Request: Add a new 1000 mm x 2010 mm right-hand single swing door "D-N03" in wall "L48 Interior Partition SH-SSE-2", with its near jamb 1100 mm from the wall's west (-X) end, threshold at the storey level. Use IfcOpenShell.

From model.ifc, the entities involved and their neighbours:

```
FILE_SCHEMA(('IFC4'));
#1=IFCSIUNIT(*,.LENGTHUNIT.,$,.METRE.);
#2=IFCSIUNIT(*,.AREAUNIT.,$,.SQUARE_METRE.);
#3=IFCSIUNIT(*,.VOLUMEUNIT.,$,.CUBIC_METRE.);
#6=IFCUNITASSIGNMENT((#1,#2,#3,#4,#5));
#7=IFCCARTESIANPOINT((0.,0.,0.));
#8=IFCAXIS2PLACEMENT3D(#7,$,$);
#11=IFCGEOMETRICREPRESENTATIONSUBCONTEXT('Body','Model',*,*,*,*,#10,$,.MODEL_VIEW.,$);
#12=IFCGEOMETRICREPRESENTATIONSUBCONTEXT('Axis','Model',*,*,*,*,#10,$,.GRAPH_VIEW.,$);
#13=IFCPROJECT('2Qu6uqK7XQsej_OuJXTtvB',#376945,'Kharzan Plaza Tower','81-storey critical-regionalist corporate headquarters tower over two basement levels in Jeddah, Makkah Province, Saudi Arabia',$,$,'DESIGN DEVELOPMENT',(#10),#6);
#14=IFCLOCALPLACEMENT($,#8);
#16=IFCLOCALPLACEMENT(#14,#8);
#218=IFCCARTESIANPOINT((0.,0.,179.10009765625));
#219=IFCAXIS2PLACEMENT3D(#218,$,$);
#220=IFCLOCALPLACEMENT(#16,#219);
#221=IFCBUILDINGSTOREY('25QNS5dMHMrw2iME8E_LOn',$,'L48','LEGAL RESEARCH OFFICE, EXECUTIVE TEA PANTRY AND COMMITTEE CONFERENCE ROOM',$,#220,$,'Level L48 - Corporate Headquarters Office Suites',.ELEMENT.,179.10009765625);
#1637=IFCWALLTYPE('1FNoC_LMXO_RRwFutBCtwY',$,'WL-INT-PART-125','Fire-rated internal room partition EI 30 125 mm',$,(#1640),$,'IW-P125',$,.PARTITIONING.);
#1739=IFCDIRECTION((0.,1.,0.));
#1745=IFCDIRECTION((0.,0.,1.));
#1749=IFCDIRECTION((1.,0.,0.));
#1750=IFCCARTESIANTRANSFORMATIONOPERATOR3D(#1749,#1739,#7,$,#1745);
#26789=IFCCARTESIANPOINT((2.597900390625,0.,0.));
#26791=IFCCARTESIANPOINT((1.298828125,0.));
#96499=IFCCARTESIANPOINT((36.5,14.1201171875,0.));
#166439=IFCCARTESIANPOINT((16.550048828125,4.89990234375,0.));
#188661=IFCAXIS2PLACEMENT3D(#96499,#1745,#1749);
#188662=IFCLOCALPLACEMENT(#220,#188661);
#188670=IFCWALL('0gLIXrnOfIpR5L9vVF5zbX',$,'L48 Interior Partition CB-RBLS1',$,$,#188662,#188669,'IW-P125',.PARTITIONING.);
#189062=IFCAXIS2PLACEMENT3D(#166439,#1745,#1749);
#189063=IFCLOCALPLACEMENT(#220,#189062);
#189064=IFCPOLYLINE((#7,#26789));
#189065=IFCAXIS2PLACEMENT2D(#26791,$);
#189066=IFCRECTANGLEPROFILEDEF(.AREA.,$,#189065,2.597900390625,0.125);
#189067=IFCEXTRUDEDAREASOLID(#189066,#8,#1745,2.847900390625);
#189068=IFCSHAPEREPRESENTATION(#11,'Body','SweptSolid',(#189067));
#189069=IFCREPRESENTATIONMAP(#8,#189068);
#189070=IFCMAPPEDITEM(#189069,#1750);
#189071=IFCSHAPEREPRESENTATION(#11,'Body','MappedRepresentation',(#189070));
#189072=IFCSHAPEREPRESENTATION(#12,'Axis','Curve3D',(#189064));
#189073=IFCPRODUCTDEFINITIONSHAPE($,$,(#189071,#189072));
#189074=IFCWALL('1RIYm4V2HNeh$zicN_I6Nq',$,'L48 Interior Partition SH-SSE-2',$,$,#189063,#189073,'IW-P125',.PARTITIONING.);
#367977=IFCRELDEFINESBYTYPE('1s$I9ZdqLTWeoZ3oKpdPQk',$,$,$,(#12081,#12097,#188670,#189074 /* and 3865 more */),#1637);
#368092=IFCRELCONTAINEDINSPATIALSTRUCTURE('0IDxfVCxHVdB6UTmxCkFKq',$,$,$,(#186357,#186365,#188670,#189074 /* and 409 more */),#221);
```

```python
import numpy as np
import ifcopenshell
import ifcopenshell.api.feature
import ifcopenshell.api.geometry
import ifcopenshell.api.root
import ifcopenshell.api.spatial
import ifcopenshell.geom
import ifcopenshell.util.element
import ifcopenshell.util.placement
import ifcopenshell.util.representation
import ifcopenshell.util.shape
import ifcopenshell.util.unit

model = ifcopenshell.open("model.ifc")
unit_scale = ifcopenshell.util.unit.calculate_unit_scale(model)
settings = ifcopenshell.geom.settings()


def volume(element):
    """Net volume in cubic metres, openings subtracted."""
    shape = ifcopenshell.geom.create_shape(settings, element)
    return ifcopenshell.util.shape.get_volume(shape.geometry)


wall = model.by_guid("1RIYm4V2HNeh$zicN_I6Nq")
storey = ifcopenshell.util.element.get_container(wall, ifc_class="IfcBuildingStorey")
context = ifcopenshell.util.representation.get_context(model, "Model", "Body", "MODEL_VIEW")
before = volume(wall)

width, height, from_end, sill = 1, 2.01, 1.1, 0.0  # metres

# The wall runs along its own X axis, and the end named is its -X end.
wall_shape = ifcopenshell.geom.create_shape(settings, wall)
x, y, z = ifcopenshell.util.shape.get_vertices(wall_shape.geometry).T
start = x.min() + from_end
face, thickness = float(y.min()), float(y.max() - y.min())
wall_matrix = ifcopenshell.util.placement.get_local_placement(wall.ObjectPlacement)
level = ifcopenshell.util.placement.get_local_placement(storey.ObjectPlacement)[2, 3]


def in_wall(x, y):
    """Placement at x, y metres in the wall's axes, at sill height."""
    matrix = wall_matrix.copy()
    matrix[:, 3] = wall_matrix @ np.array([x / unit_scale, y / unit_scale, 0.0, 1.0])
    matrix[2, 3] = level + sill / unit_scale
    return matrix


# Opening: a box that overshoots both wall faces by 50 mm.
opening = ifcopenshell.api.root.create_entity(model, ifc_class="IfcOpeningElement", predefined_type="OPENING")
box = ifcopenshell.api.geometry.add_wall_representation(
    model, context=context, length=width, height=height, thickness=thickness + 0.1
)
ifcopenshell.api.geometry.assign_representation(model, product=opening, representation=box)
ifcopenshell.api.geometry.edit_object_placement(model, product=opening, matrix=in_wall(start, face - 0.05), is_si=False)
ifcopenshell.api.feature.add_feature(model, feature=opening, element=wall)

door = ifcopenshell.api.root.create_entity(model, ifc_class="IfcDoor", name="D-N03", predefined_type="DOOR")
door.OverallWidth, door.OverallHeight = width / unit_scale, height / unit_scale
door.OperationType = "SINGLE_SWING_RIGHT"
body = ifcopenshell.api.geometry.add_door_representation(
    model,
    context=context,
    overall_width=door.OverallWidth,
    overall_height=door.OverallHeight,
    operation_type="SINGLE_SWING_RIGHT",
    lining_properties={"LiningDepth": thickness / unit_scale, "ThresholdDepth": thickness / unit_scale},
)
ifcopenshell.api.geometry.assign_representation(model, product=door, representation=body)
ifcopenshell.api.spatial.assign_container(model, products=[door], relating_structure=storey)
ifcopenshell.api.feature.add_filling(model, opening=opening, element=door)

# The lining spans the wall, so the door starts at the wall face.
ifcopenshell.api.geometry.edit_object_placement(model, product=door, matrix=in_wall(start, face), is_si=False)

after = volume(wall)

print(f"wall volume {before:.3f} -> {after:.3f} m3")

model.write("model_v2.ifc")
```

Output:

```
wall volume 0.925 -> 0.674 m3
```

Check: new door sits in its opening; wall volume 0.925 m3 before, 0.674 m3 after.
